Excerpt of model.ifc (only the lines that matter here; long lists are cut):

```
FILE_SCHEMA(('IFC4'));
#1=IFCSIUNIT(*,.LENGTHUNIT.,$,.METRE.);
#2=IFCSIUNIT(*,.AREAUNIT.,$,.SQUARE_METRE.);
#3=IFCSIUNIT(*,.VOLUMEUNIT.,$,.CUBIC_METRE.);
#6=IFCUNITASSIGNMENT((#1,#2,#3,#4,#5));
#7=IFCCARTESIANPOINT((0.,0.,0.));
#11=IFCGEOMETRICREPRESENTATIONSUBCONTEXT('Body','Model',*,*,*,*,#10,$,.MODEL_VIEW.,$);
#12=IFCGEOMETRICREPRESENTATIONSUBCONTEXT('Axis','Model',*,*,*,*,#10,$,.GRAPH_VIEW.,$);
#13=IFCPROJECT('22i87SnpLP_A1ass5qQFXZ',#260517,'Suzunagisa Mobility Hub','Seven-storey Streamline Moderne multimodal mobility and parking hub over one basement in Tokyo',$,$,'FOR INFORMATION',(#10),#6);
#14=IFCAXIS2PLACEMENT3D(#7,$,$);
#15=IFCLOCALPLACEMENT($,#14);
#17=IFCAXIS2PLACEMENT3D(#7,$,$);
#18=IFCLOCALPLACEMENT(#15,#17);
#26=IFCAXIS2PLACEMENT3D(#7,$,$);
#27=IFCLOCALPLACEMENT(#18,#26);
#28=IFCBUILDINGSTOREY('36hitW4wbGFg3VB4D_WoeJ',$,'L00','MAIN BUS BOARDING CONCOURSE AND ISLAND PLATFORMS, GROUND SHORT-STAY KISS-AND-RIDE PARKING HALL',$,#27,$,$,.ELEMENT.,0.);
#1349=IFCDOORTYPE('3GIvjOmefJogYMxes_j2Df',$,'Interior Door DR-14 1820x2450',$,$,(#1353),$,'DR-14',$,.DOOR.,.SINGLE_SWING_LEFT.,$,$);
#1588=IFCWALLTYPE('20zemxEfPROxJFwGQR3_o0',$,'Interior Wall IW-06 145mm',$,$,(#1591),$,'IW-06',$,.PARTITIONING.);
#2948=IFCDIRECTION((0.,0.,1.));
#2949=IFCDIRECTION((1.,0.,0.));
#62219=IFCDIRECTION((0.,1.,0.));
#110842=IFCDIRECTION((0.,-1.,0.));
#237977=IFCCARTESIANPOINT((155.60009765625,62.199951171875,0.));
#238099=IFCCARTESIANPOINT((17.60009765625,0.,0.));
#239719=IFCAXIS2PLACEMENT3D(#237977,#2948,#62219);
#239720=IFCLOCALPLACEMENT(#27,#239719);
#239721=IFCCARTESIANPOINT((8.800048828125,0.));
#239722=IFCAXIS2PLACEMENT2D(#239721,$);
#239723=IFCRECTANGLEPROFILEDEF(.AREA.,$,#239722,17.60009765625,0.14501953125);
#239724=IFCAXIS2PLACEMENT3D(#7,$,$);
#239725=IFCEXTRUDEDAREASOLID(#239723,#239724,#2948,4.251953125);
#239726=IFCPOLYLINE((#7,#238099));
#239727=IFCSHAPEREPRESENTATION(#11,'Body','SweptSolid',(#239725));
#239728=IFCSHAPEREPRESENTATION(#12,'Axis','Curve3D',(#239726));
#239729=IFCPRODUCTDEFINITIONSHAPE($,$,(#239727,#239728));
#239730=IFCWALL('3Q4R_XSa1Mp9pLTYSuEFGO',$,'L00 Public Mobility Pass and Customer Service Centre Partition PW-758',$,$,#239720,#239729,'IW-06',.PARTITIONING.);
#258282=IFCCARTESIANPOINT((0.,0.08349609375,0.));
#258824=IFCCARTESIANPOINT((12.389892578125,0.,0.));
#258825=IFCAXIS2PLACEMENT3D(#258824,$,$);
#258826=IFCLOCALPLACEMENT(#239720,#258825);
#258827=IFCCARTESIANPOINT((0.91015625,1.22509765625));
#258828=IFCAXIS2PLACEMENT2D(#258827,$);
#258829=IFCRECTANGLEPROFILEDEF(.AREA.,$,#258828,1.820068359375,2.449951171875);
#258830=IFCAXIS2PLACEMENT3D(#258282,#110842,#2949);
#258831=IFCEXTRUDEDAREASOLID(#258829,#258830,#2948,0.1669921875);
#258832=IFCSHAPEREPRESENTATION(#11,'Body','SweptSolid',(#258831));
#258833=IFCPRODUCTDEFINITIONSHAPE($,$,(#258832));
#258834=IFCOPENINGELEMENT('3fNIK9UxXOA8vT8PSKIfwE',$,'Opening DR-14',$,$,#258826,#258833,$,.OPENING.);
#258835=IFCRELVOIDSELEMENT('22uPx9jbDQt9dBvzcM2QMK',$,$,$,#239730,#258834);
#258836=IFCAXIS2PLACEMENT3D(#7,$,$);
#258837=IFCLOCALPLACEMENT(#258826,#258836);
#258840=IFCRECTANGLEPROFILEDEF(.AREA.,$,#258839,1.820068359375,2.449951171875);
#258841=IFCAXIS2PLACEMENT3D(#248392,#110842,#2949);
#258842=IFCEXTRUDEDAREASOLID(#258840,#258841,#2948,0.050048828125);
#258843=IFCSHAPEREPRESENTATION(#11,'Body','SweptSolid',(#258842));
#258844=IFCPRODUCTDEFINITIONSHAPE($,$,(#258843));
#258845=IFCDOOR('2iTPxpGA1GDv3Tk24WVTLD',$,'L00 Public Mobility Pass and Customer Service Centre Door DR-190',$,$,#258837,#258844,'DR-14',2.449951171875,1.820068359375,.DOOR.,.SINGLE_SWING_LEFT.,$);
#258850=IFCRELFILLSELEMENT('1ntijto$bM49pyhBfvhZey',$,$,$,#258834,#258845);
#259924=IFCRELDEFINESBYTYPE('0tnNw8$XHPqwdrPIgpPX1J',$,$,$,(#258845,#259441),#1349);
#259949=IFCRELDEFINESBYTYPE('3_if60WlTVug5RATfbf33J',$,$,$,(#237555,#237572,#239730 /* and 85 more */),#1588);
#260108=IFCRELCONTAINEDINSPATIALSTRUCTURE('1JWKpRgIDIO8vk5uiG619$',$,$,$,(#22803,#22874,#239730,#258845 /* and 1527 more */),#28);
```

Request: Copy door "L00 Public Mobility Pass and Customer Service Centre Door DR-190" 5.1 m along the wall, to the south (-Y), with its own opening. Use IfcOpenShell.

```python
import ifcopenshell
import ifcopenshell.api.feature
import ifcopenshell.api.geometry
import ifcopenshell.api.root
import ifcopenshell.geom
import ifcopenshell.util.element
import ifcopenshell.util.placement
import ifcopenshell.util.shape

model = ifcopenshell.open("model.ifc")
settings = ifcopenshell.geom.settings()


def volume(element):
    """Net volume in cubic metres, openings subtracted."""
    shape = ifcopenshell.geom.create_shape(settings, element)
    return ifcopenshell.util.shape.get_volume(shape.geometry)


door = model.by_guid("2iTPxpGA1GDv3Tk24WVTLD")
opening = door.FillsVoids[0].RelatingOpeningElement
wall = opening.VoidsElements[0].RelatingBuildingElement
before = volume(wall)
shift = ifcopenshell.util.placement.get_local_placement(wall.ObjectPlacement)[:3, 0] * -5.1

# copy_class copies the void relationship, type, container and properties, but no geometry.
new_opening = ifcopenshell.api.root.copy_class(model, product=opening)
new_opening.Representation = ifcopenshell.util.element.copy_deep(
    model, opening.Representation, exclude=["IfcGeometricRepresentationContext", "IfcRepresentationMap"]
)
new_door = ifcopenshell.api.root.copy_class(model, product=door)
new_door.Representation = ifcopenshell.util.element.copy_deep(
    model, door.Representation, exclude=["IfcGeometricRepresentationContext", "IfcRepresentationMap"]
)
new_door.Tag = None
ifcopenshell.api.feature.add_filling(model, opening=new_opening, element=new_door)

for old, new in ((opening, new_opening), (door, new_door)):
    matrix = ifcopenshell.util.placement.get_local_placement(old.ObjectPlacement)
    matrix[:3, 3] += shift
    ifcopenshell.api.geometry.edit_object_placement(model, product=new, matrix=matrix, is_si=False)

after = volume(wall)

print(f"wall volume {before:.3f} -> {after:.3f} m3")

model.write("model_rev.ifc")
```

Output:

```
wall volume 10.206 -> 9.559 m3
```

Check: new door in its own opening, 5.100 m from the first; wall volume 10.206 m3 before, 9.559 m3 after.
